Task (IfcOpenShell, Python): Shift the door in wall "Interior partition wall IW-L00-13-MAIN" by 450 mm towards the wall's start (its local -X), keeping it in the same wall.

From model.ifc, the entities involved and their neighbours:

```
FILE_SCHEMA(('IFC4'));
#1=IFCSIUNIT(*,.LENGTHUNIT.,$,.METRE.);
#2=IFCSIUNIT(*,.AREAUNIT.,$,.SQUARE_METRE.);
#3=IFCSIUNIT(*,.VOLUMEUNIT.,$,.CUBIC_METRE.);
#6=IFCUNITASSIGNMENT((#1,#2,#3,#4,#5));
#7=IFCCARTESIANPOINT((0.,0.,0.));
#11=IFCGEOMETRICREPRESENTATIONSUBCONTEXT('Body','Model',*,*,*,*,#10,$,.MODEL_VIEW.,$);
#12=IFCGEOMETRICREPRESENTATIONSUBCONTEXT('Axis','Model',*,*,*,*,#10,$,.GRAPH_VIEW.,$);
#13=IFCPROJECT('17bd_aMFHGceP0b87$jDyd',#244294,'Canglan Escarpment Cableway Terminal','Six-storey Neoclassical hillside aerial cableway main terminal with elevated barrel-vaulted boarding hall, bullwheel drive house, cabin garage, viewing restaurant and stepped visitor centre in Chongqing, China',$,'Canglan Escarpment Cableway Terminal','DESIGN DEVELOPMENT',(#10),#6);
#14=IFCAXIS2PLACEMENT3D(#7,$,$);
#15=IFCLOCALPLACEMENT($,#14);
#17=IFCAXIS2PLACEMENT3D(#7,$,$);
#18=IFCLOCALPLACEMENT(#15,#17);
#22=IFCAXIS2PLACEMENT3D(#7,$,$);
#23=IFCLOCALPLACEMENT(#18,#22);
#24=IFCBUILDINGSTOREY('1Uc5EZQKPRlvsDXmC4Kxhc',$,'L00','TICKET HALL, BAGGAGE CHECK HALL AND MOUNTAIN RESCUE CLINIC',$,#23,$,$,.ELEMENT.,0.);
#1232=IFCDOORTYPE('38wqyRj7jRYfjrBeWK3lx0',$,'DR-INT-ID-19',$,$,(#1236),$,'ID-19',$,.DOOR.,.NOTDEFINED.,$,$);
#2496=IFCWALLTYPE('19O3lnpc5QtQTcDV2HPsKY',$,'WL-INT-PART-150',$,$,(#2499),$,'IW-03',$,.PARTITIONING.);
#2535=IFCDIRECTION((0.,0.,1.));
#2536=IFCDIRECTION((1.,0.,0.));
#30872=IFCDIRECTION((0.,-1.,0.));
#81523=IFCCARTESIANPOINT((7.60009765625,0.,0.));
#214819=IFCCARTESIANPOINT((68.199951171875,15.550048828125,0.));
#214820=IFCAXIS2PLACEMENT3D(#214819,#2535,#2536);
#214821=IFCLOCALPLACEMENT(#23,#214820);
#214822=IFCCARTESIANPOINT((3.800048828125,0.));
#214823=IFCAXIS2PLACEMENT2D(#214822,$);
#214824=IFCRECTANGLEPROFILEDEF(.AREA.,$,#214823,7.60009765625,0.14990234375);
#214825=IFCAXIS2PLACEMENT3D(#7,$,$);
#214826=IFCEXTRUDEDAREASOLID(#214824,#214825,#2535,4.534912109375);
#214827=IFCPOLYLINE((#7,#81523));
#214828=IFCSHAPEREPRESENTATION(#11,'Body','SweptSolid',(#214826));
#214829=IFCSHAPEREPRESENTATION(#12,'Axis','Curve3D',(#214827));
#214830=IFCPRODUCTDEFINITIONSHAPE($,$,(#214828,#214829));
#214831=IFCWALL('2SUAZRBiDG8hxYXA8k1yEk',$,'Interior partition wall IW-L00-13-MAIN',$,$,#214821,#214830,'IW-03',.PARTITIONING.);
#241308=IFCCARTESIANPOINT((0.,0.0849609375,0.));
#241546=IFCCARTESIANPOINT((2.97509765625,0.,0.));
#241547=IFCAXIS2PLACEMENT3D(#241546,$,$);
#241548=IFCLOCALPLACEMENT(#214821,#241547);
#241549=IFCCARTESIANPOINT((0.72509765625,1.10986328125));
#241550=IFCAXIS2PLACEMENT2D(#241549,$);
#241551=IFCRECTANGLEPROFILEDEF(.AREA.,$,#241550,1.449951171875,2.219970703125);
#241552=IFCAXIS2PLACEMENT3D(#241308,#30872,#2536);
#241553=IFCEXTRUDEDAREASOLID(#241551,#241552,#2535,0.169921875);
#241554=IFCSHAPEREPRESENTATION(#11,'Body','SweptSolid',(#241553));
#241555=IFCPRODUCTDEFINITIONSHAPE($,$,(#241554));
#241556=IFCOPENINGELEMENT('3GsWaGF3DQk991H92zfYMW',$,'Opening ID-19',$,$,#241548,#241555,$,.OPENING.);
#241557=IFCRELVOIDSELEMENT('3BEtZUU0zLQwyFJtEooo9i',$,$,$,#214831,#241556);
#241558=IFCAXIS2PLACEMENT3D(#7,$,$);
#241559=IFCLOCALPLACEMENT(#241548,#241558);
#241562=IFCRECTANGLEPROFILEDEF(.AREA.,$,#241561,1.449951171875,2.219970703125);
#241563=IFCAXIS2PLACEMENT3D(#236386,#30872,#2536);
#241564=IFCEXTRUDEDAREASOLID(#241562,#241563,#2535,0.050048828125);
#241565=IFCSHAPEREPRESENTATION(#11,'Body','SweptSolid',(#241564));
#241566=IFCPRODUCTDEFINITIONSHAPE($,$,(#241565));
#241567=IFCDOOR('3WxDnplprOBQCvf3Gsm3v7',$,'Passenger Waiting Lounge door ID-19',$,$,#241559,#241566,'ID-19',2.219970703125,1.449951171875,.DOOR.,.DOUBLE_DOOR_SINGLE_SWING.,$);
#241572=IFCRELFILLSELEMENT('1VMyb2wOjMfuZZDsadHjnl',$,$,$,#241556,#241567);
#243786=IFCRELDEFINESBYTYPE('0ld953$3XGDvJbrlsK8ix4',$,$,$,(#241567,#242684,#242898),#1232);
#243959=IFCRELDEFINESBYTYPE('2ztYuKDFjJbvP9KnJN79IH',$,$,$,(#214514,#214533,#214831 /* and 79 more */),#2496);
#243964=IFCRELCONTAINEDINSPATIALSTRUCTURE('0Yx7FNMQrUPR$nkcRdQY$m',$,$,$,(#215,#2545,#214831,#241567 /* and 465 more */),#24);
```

```python
import ifcopenshell
import ifcopenshell.api.geometry
import ifcopenshell.util.placement
import ifcopenshell.util.unit

model = ifcopenshell.open("model.ifc")
unit_scale = ifcopenshell.util.unit.calculate_unit_scale(model)

door = model.by_guid("3WxDnplprOBQCvf3Gsm3v7")
opening = door.FillsVoids[0].RelatingOpeningElement
wall = opening.VoidsElements[0].RelatingBuildingElement

wall_matrix = ifcopenshell.util.placement.get_local_placement(wall.ObjectPlacement)
shift = wall_matrix[:3, 0] * -0.45 / unit_scale
before = ifcopenshell.util.placement.get_local_placement(door.ObjectPlacement)[:3, 3].copy()

# The door is placed relative to its opening, so it follows when the opening moves.
matrix = ifcopenshell.util.placement.get_local_placement(opening.ObjectPlacement)
matrix[:3, 3] += shift
ifcopenshell.api.geometry.edit_object_placement(
    model, product=opening, matrix=matrix, is_si=False, should_transform_children=True
)

after = ifcopenshell.util.placement.get_local_placement(door.ObjectPlacement)[:3, 3]
print("door moved by", (after - before).round(3) + 0.0)

model.write("model_rev.ifc")
```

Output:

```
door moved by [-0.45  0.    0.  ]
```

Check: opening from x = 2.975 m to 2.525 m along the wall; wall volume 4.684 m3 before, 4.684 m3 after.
